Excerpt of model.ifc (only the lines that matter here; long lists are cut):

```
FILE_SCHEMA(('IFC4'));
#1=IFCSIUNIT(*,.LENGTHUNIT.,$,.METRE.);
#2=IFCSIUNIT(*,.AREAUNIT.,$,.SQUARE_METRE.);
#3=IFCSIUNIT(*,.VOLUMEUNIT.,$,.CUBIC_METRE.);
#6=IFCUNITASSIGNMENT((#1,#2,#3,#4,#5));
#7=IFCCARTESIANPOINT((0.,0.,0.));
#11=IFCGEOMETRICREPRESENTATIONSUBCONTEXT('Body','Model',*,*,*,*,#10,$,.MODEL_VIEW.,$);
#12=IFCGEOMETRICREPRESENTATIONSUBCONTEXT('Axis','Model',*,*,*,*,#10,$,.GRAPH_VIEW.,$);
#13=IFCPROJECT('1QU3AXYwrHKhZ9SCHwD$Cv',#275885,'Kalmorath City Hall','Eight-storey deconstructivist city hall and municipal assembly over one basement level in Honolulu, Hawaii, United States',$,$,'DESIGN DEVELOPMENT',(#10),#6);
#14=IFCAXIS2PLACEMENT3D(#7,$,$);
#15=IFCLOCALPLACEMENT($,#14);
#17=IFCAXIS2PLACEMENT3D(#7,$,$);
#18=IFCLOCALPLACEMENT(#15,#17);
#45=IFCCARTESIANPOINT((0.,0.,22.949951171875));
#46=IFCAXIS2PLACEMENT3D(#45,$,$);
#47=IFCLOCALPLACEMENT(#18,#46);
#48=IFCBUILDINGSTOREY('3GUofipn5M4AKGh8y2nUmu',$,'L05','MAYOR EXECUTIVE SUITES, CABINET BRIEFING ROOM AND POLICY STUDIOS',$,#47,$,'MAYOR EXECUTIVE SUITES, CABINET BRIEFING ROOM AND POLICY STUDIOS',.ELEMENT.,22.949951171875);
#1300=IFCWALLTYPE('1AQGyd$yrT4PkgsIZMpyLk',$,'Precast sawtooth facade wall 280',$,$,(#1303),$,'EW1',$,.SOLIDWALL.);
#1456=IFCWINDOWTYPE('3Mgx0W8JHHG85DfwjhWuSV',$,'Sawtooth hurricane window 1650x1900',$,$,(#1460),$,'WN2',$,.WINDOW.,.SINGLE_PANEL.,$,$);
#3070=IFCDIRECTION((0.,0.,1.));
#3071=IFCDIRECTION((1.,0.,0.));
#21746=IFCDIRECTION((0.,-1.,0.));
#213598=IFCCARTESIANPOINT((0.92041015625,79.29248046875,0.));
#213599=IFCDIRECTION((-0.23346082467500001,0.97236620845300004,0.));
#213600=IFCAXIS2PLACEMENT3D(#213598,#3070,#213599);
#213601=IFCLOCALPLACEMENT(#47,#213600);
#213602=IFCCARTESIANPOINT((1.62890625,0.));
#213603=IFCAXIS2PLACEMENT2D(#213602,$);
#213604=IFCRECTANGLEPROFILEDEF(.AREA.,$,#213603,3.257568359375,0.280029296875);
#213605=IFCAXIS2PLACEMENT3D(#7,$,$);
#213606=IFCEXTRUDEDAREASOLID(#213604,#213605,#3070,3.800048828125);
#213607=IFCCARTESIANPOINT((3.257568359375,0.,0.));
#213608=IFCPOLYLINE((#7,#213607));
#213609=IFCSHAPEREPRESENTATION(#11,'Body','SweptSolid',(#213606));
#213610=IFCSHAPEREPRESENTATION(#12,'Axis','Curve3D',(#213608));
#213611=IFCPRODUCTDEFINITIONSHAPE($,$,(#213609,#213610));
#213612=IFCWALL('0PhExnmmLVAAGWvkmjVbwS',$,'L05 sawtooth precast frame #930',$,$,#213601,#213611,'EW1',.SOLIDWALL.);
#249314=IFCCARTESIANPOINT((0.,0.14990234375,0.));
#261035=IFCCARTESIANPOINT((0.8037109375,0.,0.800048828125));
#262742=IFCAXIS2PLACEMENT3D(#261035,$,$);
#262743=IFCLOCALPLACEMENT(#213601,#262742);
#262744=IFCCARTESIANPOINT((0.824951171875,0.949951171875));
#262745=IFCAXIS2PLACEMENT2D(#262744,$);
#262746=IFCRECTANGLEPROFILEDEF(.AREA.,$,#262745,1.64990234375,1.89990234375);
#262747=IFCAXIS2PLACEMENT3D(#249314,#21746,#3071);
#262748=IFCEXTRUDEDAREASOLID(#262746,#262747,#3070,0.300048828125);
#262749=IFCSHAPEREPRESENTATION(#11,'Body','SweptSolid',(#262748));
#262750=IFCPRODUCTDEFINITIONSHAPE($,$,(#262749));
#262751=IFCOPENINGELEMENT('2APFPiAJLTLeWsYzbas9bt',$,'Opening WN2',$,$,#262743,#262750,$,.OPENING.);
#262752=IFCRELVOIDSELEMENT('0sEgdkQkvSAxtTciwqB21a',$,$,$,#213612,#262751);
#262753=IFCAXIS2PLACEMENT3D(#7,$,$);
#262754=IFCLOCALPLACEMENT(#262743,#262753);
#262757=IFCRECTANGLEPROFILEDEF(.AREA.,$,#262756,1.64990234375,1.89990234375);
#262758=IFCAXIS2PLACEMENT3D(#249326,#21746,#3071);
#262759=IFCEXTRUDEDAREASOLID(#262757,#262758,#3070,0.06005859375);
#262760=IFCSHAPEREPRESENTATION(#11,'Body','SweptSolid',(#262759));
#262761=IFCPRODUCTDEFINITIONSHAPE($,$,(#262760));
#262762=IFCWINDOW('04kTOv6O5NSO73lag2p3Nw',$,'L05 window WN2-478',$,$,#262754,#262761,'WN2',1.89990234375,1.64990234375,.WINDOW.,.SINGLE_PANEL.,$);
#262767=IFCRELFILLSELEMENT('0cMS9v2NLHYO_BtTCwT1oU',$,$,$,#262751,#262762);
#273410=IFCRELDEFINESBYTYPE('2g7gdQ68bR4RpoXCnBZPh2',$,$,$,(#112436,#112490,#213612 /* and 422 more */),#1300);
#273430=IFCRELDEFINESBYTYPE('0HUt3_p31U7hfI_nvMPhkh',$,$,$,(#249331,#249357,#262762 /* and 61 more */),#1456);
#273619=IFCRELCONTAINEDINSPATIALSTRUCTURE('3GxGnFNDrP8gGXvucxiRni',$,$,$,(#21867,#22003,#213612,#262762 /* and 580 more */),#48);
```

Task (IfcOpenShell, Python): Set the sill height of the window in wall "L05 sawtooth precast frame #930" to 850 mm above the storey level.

```python
import numpy as np
import ifcopenshell
import ifcopenshell.api.geometry
import ifcopenshell.geom
import ifcopenshell.util.element
import ifcopenshell.util.placement
import ifcopenshell.util.shape
import ifcopenshell.util.unit

model = ifcopenshell.open("model.ifc")
unit_scale = ifcopenshell.util.unit.calculate_unit_scale(model)

window = model.by_guid("04kTOv6O5NSO73lag2p3Nw")
opening = window.FillsVoids[0].RelatingOpeningElement
storey = ifcopenshell.util.element.get_container(window, ifc_class="IfcBuildingStorey")
level = ifcopenshell.util.placement.get_local_placement(storey.ObjectPlacement)[2, 3]

# The opening's origin need not be at the sill, so measure its lowest point.
shape = ifcopenshell.geom.create_shape(ifcopenshell.geom.settings(), opening)
bottom = ifcopenshell.util.shape.get_shape_bottom_elevation(shape, shape.geometry) / unit_scale
dz = level + 0.85 / unit_scale - bottom

shift = np.array([0.0, 0.0, dz])
# The window is placed relative to its opening, so it follows when the opening moves.
matrix = ifcopenshell.util.placement.get_local_placement(opening.ObjectPlacement)
matrix[:3, 3] += shift
ifcopenshell.api.geometry.edit_object_placement(
    model, product=opening, matrix=matrix, is_si=False, should_transform_children=True
)

print(f"moved by {dz * unit_scale:+.3f} m")

model.write("model_rev.ifc")
```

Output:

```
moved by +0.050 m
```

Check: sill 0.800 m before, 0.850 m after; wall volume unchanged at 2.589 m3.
